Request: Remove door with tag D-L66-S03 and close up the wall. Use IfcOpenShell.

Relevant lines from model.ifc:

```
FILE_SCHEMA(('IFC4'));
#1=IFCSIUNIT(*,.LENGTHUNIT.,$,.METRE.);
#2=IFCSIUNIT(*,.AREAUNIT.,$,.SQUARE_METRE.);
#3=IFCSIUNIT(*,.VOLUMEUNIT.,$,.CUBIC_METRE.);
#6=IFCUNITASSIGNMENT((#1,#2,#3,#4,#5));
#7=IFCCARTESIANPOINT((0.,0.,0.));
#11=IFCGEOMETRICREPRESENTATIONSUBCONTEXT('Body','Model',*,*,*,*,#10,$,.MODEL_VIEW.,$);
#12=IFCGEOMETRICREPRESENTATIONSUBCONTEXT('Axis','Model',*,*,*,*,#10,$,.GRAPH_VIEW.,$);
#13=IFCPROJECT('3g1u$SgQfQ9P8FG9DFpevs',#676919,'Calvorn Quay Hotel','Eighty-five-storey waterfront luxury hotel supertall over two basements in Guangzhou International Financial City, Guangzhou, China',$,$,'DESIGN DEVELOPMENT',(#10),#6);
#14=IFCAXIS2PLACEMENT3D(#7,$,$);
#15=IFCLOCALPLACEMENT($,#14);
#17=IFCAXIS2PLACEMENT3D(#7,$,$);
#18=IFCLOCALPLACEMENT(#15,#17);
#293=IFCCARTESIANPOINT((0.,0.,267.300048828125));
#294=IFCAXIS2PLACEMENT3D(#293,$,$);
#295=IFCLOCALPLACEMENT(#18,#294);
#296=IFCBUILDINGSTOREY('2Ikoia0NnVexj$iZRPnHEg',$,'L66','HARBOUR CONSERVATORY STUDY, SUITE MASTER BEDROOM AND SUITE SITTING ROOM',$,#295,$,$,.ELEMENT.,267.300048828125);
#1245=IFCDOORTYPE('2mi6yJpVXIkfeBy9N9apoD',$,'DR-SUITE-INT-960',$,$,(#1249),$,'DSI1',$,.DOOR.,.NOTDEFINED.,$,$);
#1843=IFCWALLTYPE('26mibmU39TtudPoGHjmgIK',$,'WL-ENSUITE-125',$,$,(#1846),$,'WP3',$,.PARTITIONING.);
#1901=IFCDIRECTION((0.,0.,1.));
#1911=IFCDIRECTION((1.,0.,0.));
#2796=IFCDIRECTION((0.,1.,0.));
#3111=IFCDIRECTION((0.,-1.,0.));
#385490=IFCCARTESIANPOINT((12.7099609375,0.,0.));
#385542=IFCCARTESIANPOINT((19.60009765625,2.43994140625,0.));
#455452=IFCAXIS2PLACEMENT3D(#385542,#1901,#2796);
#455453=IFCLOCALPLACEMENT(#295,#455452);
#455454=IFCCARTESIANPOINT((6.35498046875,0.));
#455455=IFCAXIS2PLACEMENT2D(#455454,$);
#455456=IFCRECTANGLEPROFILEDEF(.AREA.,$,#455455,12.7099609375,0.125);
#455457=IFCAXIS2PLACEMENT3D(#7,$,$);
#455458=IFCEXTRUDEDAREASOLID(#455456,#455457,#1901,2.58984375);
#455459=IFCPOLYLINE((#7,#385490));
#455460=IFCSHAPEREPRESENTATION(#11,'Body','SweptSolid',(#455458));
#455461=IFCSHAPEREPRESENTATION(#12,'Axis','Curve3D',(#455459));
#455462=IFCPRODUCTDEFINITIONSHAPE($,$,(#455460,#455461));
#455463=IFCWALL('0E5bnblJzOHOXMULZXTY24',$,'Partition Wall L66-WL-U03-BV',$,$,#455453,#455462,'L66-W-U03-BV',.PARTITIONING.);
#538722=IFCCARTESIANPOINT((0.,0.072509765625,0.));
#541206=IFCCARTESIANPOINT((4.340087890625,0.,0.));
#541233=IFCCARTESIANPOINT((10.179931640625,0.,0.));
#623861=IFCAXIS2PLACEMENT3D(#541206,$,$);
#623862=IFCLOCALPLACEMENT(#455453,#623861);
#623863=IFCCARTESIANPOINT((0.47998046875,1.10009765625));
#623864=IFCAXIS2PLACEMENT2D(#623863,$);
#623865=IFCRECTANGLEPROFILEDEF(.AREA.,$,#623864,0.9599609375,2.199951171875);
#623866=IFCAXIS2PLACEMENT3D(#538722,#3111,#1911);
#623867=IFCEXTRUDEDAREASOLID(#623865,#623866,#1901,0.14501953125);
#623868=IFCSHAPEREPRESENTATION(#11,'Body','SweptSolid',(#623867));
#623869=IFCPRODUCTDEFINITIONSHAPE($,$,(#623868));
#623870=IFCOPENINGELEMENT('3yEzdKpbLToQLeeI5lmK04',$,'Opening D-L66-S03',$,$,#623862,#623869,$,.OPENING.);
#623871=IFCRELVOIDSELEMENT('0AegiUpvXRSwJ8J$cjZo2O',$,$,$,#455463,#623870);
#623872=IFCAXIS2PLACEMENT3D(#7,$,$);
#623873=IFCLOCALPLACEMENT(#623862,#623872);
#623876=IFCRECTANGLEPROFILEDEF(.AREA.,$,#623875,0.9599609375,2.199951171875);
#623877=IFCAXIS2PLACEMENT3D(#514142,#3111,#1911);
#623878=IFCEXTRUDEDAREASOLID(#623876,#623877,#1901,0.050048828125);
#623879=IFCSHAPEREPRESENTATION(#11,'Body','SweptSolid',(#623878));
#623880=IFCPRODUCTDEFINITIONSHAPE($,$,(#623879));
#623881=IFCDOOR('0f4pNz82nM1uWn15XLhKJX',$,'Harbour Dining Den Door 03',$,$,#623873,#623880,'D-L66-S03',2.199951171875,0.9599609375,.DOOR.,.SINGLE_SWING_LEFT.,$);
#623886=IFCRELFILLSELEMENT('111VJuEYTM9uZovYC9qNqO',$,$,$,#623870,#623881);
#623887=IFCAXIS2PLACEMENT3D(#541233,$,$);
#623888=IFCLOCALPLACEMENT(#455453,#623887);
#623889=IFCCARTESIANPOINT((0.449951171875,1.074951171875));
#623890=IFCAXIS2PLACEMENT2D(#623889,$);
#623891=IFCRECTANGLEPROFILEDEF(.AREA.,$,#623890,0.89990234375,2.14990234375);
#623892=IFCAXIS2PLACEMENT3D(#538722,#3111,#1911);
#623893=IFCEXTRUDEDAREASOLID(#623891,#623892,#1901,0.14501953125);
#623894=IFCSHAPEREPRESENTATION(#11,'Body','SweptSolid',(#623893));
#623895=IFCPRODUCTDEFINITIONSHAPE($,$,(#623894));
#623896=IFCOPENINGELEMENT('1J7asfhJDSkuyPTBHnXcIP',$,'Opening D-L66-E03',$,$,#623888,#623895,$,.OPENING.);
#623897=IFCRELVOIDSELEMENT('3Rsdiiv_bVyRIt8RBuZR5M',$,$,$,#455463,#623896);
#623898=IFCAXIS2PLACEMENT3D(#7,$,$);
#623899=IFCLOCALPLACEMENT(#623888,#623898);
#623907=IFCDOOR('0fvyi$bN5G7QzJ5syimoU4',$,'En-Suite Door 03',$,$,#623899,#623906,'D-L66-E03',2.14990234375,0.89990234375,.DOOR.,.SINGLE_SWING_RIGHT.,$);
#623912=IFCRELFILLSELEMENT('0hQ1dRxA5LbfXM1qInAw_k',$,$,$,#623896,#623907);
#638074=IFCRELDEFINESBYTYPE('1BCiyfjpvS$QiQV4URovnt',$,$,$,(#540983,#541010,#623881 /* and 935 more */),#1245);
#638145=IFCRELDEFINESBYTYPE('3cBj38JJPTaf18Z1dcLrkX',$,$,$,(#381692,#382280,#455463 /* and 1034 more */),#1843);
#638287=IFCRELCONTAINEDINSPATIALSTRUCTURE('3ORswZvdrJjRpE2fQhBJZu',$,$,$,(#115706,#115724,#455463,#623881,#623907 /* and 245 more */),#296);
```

```python
import ifcopenshell
import ifcopenshell.api.feature
import ifcopenshell.api.root
import ifcopenshell.geom
import ifcopenshell.util.shape

model = ifcopenshell.open("model.ifc")
settings = ifcopenshell.geom.settings()


def volume(element):
    """Net volume in cubic metres, openings subtracted."""
    shape = ifcopenshell.geom.create_shape(settings, element)
    return ifcopenshell.util.shape.get_volume(shape.geometry)


door = model.by_guid("0f4pNz82nM1uWn15XLhKJX")
opening = door.FillsVoids[0].RelatingOpeningElement
wall = opening.VoidsElements[0].RelatingBuildingElement
before = volume(wall)

ifcopenshell.api.root.remove_product(model, product=door)
ifcopenshell.api.feature.remove_feature(model, feature=opening)

after = volume(wall)

print(f"wall volume {before:.3f} -> {after:.3f} m3")

model.write("model_v2.ifc")
```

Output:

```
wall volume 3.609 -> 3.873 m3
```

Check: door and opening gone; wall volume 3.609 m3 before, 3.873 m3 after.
